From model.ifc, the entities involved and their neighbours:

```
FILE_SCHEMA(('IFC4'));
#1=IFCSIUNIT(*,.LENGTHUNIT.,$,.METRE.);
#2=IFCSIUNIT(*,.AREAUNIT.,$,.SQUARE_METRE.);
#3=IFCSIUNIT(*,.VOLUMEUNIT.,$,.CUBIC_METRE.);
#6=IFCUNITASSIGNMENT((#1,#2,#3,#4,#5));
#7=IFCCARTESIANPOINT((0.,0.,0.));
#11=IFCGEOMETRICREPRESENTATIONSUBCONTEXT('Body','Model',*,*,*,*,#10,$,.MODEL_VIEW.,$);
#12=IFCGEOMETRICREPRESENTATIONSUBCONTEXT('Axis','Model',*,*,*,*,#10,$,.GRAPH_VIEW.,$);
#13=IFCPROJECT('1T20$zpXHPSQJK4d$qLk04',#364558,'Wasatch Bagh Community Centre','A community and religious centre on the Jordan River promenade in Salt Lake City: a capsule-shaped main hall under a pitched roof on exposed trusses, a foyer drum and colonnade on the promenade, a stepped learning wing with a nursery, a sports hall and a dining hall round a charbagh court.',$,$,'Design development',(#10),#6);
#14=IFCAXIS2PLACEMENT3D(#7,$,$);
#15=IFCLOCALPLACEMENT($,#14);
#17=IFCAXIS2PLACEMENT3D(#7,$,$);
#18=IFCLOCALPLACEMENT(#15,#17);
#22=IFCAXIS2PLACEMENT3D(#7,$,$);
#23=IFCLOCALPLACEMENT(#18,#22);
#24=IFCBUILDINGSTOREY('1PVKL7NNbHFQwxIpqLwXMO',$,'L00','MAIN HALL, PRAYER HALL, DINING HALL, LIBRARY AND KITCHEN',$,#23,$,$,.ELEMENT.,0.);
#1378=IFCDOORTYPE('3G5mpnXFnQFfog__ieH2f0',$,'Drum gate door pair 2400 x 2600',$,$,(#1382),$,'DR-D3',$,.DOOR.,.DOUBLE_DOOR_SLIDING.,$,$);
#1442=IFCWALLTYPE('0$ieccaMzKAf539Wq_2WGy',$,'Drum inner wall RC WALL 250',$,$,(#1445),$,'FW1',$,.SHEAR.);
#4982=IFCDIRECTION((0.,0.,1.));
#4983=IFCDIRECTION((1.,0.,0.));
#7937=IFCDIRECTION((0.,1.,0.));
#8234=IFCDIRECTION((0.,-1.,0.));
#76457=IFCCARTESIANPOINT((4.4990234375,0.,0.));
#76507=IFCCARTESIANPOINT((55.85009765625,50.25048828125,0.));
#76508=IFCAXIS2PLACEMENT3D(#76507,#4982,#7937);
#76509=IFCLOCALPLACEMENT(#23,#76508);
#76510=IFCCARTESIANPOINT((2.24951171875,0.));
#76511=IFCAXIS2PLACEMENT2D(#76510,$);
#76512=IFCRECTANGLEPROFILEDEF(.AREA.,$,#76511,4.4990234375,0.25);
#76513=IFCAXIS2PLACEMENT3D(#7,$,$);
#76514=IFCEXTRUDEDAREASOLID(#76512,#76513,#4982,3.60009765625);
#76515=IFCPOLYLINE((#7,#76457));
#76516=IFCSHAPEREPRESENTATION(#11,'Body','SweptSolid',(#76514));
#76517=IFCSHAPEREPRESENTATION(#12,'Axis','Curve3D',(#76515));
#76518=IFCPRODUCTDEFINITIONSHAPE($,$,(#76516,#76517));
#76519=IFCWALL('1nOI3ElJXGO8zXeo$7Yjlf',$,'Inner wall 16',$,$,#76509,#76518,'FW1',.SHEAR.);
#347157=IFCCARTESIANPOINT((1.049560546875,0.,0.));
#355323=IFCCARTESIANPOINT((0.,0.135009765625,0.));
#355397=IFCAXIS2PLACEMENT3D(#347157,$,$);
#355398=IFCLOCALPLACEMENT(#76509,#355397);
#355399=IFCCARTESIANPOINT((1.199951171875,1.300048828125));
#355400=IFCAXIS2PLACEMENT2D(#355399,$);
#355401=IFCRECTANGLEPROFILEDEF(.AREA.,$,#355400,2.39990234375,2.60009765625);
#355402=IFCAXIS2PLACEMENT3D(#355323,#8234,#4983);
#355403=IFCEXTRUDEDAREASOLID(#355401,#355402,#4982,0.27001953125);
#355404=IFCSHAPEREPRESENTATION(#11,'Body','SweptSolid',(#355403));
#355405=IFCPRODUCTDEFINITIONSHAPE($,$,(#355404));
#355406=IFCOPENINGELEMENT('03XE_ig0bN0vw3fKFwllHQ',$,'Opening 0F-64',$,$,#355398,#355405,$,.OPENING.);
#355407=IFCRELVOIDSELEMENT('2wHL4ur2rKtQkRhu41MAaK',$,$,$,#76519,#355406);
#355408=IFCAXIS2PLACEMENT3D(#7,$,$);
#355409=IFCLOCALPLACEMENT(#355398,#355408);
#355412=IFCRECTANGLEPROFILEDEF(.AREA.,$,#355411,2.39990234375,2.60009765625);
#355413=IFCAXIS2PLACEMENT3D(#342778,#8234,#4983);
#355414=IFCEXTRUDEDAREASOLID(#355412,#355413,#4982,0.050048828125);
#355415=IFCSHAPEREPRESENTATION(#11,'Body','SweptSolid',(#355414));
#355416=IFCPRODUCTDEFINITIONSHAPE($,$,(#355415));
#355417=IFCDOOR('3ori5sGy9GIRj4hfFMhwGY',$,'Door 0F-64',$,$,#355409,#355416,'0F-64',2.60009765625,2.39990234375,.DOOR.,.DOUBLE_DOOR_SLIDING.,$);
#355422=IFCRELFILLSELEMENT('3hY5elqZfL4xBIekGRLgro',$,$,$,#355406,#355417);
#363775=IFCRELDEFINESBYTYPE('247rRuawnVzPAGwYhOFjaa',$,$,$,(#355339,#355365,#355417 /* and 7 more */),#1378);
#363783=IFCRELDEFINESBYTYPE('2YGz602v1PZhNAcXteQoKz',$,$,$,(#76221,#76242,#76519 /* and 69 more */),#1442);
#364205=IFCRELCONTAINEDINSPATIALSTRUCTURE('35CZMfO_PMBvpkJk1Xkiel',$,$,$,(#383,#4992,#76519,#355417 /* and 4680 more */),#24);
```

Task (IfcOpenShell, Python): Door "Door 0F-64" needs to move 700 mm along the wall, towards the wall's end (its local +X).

```python
import ifcopenshell
import ifcopenshell.api.geometry
import ifcopenshell.util.placement
import ifcopenshell.util.unit

model = ifcopenshell.open("model.ifc")
unit_scale = ifcopenshell.util.unit.calculate_unit_scale(model)

door = model.by_id(355417)
opening = door.FillsVoids[0].RelatingOpeningElement
wall = opening.VoidsElements[0].RelatingBuildingElement

wall_matrix = ifcopenshell.util.placement.get_local_placement(wall.ObjectPlacement)
shift = wall_matrix[:3, 0] * 0.7 / unit_scale
before = ifcopenshell.util.placement.get_local_placement(door.ObjectPlacement)[:3, 3].copy()

# The door is placed relative to its opening, so it follows when the opening moves.
matrix = ifcopenshell.util.placement.get_local_placement(opening.ObjectPlacement)
matrix[:3, 3] += shift
ifcopenshell.api.geometry.edit_object_placement(
    model, product=opening, matrix=matrix, is_si=False, should_transform_children=True
)

after = ifcopenshell.util.placement.get_local_placement(door.ObjectPlacement)[:3, 3]
print("door moved by", (after - before).round(3) + 0.0)

model.write("model_rev.ifc")
```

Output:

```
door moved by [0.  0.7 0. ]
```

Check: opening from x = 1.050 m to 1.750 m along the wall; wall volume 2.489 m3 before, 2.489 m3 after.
